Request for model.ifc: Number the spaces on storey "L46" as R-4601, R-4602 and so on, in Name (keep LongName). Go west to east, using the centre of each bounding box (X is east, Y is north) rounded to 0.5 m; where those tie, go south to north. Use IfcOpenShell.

First a look at what the model holds.

```python
import ifcopenshell
import ifcopenshell.util.element
import ifcopenshell.util.placement

model = ifcopenshell.open("model.ifc")
print(model.schema)
storey = next(s for s in model.by_type("IfcBuildingStorey") if s.Name == "L46")
spaces = [e for e in ifcopenshell.util.element.get_decomposition(storey) if e.is_a("IfcSpace")]
for e in sorted(spaces, key=lambda e: e.id()):
    origin = ifcopenshell.util.placement.get_local_placement(e.ObjectPlacement)[:3, 3]
    print(e.id(), e.Name, e.LongName, origin.round(2) + 0.0, sep=" | ")
```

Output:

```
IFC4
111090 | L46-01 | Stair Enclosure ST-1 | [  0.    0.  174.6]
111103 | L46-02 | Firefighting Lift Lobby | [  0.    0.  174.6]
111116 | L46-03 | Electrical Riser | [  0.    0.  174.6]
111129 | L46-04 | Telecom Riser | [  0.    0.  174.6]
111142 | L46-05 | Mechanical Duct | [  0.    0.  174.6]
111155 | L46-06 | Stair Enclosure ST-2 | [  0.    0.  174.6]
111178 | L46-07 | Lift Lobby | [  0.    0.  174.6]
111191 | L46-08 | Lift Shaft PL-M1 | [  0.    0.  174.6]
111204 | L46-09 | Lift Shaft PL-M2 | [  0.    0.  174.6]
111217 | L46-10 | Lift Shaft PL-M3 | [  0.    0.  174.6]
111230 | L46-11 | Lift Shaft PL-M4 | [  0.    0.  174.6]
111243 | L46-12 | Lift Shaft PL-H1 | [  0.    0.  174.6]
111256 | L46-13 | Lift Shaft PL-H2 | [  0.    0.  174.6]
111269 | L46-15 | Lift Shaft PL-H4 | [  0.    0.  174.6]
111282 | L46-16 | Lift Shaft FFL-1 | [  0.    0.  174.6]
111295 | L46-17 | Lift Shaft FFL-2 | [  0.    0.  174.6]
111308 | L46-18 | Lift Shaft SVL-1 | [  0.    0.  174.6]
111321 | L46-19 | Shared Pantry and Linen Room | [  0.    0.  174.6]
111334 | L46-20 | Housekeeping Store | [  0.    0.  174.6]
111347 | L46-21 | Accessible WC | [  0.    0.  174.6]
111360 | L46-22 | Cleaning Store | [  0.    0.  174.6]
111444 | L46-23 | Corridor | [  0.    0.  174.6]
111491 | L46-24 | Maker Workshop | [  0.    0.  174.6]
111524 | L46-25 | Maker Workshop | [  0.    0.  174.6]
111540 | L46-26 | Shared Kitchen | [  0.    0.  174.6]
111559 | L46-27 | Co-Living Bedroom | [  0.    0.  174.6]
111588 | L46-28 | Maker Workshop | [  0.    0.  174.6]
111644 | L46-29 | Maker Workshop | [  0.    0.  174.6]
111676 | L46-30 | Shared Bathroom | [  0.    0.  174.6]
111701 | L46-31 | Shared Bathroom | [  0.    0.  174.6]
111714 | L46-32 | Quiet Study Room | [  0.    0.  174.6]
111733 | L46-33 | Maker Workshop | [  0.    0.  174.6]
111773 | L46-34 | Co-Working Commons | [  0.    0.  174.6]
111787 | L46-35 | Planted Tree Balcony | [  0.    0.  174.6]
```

```python
import ifcopenshell
import ifcopenshell.geom
import ifcopenshell.util.element
import ifcopenshell.util.shape

model = ifcopenshell.open("model.ifc")
settings = ifcopenshell.geom.settings()
settings.set("use-world-coords", True)


def centre(element):
    shape = ifcopenshell.geom.create_shape(settings, element)
    return ifcopenshell.util.shape.get_bbox_centroid(shape.geometry)


storey = next(s for s in model.by_type("IfcBuildingStorey") if s.Name == "L46")
spaces = [e for e in ifcopenshell.util.element.get_decomposition(storey) if e.is_a("IfcSpace")]

# Insertion points can sit at a corner or the storey origin, so sort by the geometry (in metres).
centres = {e: centre(e) for e in spaces}
spaces.sort(key=lambda e: (round(centres[e][0] / 0.5), centres[e][1]))

for i, e in enumerate(spaces, start=1):
    number = f"R-46{i:02d}"
    e.Name = number
    print(e.id(), number)

model.write("model_rev.ifc")
```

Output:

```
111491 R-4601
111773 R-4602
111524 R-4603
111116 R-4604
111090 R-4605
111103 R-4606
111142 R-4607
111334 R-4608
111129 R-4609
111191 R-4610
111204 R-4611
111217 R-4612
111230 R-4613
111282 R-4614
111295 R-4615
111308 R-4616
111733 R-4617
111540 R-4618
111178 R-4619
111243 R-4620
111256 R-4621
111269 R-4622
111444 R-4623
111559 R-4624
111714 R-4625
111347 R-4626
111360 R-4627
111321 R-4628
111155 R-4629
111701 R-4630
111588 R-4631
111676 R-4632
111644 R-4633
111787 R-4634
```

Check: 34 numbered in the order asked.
